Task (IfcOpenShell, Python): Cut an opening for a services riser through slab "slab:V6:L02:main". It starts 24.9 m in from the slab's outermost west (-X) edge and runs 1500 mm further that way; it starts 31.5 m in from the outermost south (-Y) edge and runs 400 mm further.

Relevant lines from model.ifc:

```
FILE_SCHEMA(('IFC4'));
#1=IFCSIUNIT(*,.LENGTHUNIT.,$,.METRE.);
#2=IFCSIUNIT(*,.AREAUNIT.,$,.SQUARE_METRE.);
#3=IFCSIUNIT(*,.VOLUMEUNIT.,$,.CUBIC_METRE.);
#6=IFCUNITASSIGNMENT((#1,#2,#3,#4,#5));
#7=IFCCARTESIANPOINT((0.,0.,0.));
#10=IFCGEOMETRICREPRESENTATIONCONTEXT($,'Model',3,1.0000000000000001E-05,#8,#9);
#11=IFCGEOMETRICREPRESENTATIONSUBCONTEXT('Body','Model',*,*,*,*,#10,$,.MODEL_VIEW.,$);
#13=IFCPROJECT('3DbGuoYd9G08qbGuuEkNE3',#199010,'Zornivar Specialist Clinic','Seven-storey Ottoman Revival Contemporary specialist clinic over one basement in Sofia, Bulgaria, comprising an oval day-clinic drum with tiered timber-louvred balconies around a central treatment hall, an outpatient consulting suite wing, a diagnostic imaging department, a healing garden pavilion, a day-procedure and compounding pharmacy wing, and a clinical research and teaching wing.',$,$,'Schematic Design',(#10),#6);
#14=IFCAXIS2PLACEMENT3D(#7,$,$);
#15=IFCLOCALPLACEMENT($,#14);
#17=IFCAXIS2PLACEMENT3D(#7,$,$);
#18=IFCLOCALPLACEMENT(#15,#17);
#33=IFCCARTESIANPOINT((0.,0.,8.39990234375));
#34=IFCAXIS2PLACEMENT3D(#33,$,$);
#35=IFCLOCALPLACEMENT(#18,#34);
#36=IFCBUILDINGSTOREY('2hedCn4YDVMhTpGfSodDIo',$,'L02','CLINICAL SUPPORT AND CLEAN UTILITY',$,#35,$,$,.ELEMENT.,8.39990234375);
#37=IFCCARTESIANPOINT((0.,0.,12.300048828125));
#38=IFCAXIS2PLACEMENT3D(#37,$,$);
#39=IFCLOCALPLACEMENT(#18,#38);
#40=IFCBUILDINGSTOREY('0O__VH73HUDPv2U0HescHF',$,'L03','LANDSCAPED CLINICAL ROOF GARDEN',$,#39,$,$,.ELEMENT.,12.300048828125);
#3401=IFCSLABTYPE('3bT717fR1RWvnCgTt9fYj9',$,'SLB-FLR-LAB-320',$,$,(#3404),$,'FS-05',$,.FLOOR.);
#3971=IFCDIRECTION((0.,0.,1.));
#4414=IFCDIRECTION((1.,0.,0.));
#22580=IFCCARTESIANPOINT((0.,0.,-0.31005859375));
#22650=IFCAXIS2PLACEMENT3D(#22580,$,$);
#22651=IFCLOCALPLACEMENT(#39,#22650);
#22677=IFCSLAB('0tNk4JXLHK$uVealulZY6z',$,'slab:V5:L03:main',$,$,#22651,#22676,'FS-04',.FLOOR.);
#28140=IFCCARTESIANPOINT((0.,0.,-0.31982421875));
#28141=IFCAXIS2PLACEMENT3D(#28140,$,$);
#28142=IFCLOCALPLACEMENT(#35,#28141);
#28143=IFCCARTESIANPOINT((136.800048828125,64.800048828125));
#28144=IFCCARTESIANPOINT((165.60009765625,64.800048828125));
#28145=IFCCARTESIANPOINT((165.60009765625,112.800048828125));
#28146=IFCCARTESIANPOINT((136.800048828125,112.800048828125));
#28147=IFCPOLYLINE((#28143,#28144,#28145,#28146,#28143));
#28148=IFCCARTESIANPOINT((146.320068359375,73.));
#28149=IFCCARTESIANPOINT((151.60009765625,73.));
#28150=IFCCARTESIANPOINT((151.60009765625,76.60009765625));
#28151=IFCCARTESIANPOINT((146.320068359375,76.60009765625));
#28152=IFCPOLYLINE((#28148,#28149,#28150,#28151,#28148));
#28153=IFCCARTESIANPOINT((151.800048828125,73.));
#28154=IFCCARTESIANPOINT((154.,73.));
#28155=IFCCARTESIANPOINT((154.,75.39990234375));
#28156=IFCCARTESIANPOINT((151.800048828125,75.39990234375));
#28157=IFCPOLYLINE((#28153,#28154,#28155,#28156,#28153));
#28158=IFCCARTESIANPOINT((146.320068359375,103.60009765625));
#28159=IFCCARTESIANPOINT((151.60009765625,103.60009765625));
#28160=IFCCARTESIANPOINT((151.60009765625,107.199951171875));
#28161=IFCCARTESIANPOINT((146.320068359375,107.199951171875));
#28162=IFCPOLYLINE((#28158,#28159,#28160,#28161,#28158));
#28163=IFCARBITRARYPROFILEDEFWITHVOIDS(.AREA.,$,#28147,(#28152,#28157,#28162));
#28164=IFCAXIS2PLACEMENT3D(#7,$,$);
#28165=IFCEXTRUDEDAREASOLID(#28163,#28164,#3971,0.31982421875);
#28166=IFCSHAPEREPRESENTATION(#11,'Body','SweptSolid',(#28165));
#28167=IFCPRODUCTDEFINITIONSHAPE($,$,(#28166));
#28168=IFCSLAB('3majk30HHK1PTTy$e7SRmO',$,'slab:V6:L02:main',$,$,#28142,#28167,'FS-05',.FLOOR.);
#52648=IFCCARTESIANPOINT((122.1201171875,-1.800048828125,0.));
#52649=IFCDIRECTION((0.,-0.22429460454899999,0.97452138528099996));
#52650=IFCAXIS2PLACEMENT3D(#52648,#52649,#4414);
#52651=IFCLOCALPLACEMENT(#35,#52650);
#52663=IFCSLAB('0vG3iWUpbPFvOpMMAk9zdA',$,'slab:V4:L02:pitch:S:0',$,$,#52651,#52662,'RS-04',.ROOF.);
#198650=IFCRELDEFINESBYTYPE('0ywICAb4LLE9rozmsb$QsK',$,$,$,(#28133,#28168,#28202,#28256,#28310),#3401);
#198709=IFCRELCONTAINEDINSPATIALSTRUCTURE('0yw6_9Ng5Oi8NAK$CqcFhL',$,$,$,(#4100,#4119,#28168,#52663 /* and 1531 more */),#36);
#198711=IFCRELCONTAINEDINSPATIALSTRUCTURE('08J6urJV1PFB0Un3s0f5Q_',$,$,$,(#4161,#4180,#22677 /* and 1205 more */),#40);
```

```python
import numpy as np
import ifcopenshell
import ifcopenshell.api.feature
import ifcopenshell.api.geometry
import ifcopenshell.api.root
import ifcopenshell.geom
import ifcopenshell.util.placement
import ifcopenshell.util.representation
import ifcopenshell.util.shape
import ifcopenshell.util.unit

model = ifcopenshell.open("model.ifc")
unit_scale = ifcopenshell.util.unit.calculate_unit_scale(model)
settings = ifcopenshell.geom.settings()


def volume(element):
    """Net volume in cubic metres, openings subtracted."""
    shape = ifcopenshell.geom.create_shape(settings, element)
    return ifcopenshell.util.shape.get_volume(shape.geometry)


slab = model.by_guid("3majk30HHK1PTTy$e7SRmO")
before = volume(slab)

# Extent in the slab's own axes, in metres. The edges named are its -X and -Y sides.
slab_shape = ifcopenshell.geom.create_shape(settings, slab)
vertices = ifcopenshell.util.shape.get_vertices(slab_shape.geometry)
x_min, y_min, bottom = vertices.min(axis=0)
top = vertices[:, 2].max()

opening = ifcopenshell.api.root.create_entity(model, ifc_class="IfcOpeningElement", name="Services riser opening", predefined_type="OPENING")
context = ifcopenshell.util.representation.get_context(model, "Model", "Body", "MODEL_VIEW")
width, depth = 1.5, 0.4
outline = [(0.0, 0.0), (width, 0.0), (width, depth), (0.0, depth), (0.0, 0.0)]
# Overshoot both faces by 50 mm so the cut is clean.
shape = ifcopenshell.api.geometry.add_slab_representation(
    model, context=context, depth=top - bottom + 0.1, polyline=outline
)
ifcopenshell.api.geometry.assign_representation(model, product=opening, representation=shape)

matrix = ifcopenshell.util.placement.get_local_placement(slab.ObjectPlacement)
matrix[:, 3] = matrix @ np.append(np.array([x_min + 24.9, y_min + 31.5, bottom - 0.05]) / unit_scale, 1.0)
ifcopenshell.api.geometry.edit_object_placement(model, product=opening, matrix=matrix, is_si=False)
ifcopenshell.api.feature.add_feature(model, feature=opening, element=slab)

after = volume(slab)

print(f"slab volume {before:.3f} -> {after:.3f} m3")

model.write("model_rev.ifc")
```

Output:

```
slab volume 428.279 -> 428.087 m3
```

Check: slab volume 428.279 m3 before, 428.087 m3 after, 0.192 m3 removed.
